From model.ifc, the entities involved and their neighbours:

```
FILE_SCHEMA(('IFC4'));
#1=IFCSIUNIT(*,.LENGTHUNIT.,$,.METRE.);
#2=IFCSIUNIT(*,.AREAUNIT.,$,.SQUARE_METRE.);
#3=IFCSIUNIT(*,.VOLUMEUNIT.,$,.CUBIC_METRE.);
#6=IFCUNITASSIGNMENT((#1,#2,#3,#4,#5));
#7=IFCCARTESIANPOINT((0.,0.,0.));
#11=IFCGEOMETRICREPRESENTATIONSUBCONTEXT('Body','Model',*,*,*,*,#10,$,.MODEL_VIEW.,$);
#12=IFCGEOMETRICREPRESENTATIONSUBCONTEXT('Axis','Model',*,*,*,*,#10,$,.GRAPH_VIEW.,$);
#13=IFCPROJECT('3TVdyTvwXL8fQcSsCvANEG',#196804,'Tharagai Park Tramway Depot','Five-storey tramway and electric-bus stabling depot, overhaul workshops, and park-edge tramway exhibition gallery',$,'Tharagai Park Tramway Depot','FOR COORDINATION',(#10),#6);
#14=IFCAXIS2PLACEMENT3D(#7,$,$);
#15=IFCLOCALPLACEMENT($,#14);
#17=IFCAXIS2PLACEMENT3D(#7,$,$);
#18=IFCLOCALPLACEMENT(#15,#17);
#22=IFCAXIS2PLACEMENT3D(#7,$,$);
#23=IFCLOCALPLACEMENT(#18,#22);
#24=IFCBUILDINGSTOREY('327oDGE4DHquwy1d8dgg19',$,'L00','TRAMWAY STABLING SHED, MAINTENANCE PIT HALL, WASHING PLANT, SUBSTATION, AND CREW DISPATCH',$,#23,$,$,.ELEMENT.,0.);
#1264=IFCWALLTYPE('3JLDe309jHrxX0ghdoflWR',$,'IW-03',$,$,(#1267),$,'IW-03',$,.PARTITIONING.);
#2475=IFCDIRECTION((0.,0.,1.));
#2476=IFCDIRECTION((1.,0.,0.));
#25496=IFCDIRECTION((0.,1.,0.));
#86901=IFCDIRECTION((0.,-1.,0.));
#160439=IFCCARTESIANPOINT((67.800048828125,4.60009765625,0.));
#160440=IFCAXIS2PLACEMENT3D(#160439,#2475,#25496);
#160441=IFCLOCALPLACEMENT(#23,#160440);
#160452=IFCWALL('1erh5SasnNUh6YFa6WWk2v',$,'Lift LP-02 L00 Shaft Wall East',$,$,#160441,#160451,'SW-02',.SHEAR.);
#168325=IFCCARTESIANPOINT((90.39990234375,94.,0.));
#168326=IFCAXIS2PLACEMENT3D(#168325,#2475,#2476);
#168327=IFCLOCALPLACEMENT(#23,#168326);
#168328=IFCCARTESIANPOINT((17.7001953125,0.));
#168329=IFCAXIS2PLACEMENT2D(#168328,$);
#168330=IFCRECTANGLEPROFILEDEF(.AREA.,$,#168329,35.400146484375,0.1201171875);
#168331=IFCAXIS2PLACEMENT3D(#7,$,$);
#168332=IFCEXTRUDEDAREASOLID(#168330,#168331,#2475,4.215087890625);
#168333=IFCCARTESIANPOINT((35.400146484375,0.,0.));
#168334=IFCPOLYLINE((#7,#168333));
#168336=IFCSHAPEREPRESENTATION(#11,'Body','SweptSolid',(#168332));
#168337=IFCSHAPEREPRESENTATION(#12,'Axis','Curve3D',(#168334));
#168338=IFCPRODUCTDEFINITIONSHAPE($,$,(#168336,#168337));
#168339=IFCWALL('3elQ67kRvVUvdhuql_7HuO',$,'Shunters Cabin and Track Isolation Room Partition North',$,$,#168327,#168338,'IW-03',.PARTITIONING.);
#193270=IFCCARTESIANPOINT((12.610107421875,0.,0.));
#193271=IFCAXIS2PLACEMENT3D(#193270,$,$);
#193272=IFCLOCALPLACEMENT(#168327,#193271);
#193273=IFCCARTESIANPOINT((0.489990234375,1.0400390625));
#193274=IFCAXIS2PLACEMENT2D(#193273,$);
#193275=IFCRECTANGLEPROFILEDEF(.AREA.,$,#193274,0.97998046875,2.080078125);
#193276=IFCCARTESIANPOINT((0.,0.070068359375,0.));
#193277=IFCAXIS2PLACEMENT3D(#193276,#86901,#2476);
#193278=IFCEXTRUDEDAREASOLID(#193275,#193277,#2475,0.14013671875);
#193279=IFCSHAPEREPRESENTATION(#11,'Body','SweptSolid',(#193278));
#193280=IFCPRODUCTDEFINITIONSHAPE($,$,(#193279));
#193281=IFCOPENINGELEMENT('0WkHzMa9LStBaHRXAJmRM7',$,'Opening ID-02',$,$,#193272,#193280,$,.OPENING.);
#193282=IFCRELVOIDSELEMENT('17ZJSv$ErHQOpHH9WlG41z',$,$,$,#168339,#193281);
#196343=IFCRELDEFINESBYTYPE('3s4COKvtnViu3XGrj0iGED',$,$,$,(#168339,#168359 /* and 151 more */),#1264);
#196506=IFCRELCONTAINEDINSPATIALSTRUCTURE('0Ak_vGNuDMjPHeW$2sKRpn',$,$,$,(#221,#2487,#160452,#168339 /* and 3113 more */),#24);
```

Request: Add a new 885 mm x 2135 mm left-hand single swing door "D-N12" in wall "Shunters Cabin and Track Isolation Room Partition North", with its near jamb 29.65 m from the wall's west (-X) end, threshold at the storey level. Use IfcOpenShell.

```python
import numpy as np
import ifcopenshell
import ifcopenshell.api.feature
import ifcopenshell.api.geometry
import ifcopenshell.api.root
import ifcopenshell.api.spatial
import ifcopenshell.geom
import ifcopenshell.util.element
import ifcopenshell.util.placement
import ifcopenshell.util.representation
import ifcopenshell.util.shape
import ifcopenshell.util.unit

model = ifcopenshell.open("model.ifc")
unit_scale = ifcopenshell.util.unit.calculate_unit_scale(model)
settings = ifcopenshell.geom.settings()


def volume(element):
    """Net volume in cubic metres, openings subtracted."""
    shape = ifcopenshell.geom.create_shape(settings, element)
    return ifcopenshell.util.shape.get_volume(shape.geometry)


wall = model.by_guid("3elQ67kRvVUvdhuql_7HuO")
storey = ifcopenshell.util.element.get_container(wall, ifc_class="IfcBuildingStorey")
context = ifcopenshell.util.representation.get_context(model, "Model", "Body", "MODEL_VIEW")
before = volume(wall)

width, height, from_end, sill = 0.885, 2.135, 29.65, 0.0  # metres

# The wall runs along its own X axis, and the end named is its -X end.
wall_shape = ifcopenshell.geom.create_shape(settings, wall)
x, y, z = ifcopenshell.util.shape.get_vertices(wall_shape.geometry).T
start = x.min() + from_end
face, thickness = float(y.min()), float(y.max() - y.min())
wall_matrix = ifcopenshell.util.placement.get_local_placement(wall.ObjectPlacement)
level = ifcopenshell.util.placement.get_local_placement(storey.ObjectPlacement)[2, 3]


def in_wall(x, y):
    """Placement at x, y metres in the wall's axes, at sill height."""
    matrix = wall_matrix.copy()
    matrix[:, 3] = wall_matrix @ np.array([x / unit_scale, y / unit_scale, 0.0, 1.0])
    matrix[2, 3] = level + sill / unit_scale
    return matrix


# Opening: a box that overshoots both wall faces by 50 mm.
opening = ifcopenshell.api.root.create_entity(model, ifc_class="IfcOpeningElement", predefined_type="OPENING")
box = ifcopenshell.api.geometry.add_wall_representation(
    model, context=context, length=width, height=height, thickness=thickness + 0.1
)
ifcopenshell.api.geometry.assign_representation(model, product=opening, representation=box)
ifcopenshell.api.geometry.edit_object_placement(model, product=opening, matrix=in_wall(start, face - 0.05), is_si=False)
ifcopenshell.api.feature.add_feature(model, feature=opening, element=wall)

door = ifcopenshell.api.root.create_entity(model, ifc_class="IfcDoor", name="D-N12", predefined_type="DOOR")
door.OverallWidth, door.OverallHeight = width / unit_scale, height / unit_scale
door.OperationType = "SINGLE_SWING_LEFT"
body = ifcopenshell.api.geometry.add_door_representation(
    model,
    context=context,
    overall_width=door.OverallWidth,
    overall_height=door.OverallHeight,
    operation_type="SINGLE_SWING_LEFT",
    lining_properties={"LiningDepth": thickness / unit_scale, "ThresholdDepth": thickness / unit_scale},
)
ifcopenshell.api.geometry.assign_representation(model, product=door, representation=body)
ifcopenshell.api.spatial.assign_container(model, products=[door], relating_structure=storey)
ifcopenshell.api.feature.add_filling(model, opening=opening, element=door)

# The lining spans the wall, so the door starts at the wall face.
ifcopenshell.api.geometry.edit_object_placement(model, product=door, matrix=in_wall(start, face), is_si=False)

after = volume(wall)

print(f"wall volume {before:.3f} -> {after:.3f} m3")

model.write("model-out.ifc")
```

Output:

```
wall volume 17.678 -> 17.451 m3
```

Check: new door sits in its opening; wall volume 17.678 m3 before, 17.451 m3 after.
